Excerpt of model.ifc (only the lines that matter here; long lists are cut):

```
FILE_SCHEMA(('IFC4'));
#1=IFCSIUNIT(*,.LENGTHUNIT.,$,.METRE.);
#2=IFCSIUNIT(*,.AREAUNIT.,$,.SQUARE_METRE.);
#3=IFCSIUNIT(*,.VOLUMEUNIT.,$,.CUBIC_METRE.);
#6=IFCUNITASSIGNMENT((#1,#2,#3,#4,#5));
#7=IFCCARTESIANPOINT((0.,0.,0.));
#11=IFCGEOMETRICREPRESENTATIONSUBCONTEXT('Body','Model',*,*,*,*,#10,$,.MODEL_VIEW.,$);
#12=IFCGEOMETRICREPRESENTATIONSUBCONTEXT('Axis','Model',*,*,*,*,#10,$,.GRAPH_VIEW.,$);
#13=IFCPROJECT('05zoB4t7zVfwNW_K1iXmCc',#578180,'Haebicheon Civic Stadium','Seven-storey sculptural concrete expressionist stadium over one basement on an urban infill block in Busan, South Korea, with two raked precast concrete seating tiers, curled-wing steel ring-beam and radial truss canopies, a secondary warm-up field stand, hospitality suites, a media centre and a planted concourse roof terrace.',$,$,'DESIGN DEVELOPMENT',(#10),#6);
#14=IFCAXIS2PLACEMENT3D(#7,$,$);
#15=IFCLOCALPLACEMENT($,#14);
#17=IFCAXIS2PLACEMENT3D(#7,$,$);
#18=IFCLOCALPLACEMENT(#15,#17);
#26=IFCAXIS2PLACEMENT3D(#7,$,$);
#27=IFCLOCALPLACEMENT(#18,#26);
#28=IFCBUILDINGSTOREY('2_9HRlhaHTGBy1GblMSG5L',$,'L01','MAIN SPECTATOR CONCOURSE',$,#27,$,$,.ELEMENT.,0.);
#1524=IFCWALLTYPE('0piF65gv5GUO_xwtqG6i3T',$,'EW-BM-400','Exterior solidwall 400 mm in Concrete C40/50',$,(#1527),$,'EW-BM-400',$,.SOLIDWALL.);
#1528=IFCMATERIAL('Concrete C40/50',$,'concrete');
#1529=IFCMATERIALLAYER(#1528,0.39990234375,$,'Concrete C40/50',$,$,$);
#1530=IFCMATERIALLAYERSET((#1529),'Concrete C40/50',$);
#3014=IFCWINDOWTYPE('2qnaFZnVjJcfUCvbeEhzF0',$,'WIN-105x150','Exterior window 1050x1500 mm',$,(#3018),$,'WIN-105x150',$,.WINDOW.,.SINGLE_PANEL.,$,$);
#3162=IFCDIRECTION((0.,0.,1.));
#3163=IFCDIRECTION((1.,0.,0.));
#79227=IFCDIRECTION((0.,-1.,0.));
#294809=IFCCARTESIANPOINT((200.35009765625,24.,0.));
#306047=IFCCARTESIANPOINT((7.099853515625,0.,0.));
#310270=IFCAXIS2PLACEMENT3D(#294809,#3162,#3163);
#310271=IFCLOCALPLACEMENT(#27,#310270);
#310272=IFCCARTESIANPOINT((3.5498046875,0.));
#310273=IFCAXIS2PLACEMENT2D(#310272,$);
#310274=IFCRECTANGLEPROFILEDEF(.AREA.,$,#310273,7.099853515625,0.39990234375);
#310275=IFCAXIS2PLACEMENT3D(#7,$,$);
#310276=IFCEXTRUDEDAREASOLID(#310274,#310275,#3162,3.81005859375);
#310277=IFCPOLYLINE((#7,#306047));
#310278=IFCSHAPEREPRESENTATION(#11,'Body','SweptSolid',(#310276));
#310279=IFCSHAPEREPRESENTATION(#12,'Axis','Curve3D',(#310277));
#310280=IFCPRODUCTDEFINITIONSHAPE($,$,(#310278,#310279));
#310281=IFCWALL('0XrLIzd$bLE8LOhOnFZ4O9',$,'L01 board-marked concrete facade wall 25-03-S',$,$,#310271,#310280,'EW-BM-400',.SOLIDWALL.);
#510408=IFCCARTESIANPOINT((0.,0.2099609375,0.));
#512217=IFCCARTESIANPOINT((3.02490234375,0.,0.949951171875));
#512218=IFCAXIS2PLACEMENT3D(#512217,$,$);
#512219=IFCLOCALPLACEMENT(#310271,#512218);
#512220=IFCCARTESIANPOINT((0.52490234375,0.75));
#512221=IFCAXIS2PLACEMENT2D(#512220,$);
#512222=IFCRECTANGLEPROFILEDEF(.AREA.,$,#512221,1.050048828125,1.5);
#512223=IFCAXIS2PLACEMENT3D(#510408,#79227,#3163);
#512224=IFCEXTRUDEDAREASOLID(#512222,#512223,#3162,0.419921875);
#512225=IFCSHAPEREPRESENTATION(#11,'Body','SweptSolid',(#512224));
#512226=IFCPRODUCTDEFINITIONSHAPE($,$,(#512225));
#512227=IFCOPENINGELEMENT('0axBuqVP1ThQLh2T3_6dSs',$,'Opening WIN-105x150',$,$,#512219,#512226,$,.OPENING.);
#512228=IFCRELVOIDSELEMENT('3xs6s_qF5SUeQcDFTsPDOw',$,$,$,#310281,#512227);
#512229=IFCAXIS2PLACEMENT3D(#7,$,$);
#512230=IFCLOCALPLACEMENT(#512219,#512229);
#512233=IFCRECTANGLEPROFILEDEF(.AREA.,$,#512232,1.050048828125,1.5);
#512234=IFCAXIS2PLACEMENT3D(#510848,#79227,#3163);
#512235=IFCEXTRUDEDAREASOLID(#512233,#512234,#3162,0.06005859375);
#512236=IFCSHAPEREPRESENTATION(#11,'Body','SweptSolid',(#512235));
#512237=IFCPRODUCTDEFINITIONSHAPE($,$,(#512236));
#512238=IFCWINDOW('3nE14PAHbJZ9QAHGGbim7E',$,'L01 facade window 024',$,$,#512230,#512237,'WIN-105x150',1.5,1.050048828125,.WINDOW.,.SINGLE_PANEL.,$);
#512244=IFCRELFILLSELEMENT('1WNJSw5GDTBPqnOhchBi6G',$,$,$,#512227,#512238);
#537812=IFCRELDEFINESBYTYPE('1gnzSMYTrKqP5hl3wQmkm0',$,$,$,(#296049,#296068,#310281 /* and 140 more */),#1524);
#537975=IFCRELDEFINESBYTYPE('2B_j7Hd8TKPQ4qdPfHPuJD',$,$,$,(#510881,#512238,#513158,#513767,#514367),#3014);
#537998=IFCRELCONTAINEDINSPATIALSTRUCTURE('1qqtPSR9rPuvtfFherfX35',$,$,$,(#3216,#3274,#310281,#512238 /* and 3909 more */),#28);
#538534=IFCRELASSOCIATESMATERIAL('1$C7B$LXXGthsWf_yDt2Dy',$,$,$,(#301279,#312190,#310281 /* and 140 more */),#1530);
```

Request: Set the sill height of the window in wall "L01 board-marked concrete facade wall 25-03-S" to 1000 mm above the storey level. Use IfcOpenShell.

```python
import numpy as np
import ifcopenshell
import ifcopenshell.api.geometry
import ifcopenshell.geom
import ifcopenshell.util.element
import ifcopenshell.util.placement
import ifcopenshell.util.shape
import ifcopenshell.util.unit

model = ifcopenshell.open("model.ifc")
unit_scale = ifcopenshell.util.unit.calculate_unit_scale(model)

window = model.by_guid("3nE14PAHbJZ9QAHGGbim7E")
opening = window.FillsVoids[0].RelatingOpeningElement
storey = ifcopenshell.util.element.get_container(window, ifc_class="IfcBuildingStorey")
level = ifcopenshell.util.placement.get_local_placement(storey.ObjectPlacement)[2, 3]

# The opening's origin need not be at the sill, so measure its lowest point.
shape = ifcopenshell.geom.create_shape(ifcopenshell.geom.settings(), opening)
bottom = ifcopenshell.util.shape.get_shape_bottom_elevation(shape, shape.geometry) / unit_scale
dz = level + 1 / unit_scale - bottom

shift = np.array([0.0, 0.0, dz])
# The window is placed relative to its opening, so it follows when the opening moves.
matrix = ifcopenshell.util.placement.get_local_placement(opening.ObjectPlacement)
matrix[:3, 3] += shift
ifcopenshell.api.geometry.edit_object_placement(
    model, product=opening, matrix=matrix, is_si=False, should_transform_children=True
)

print(f"moved by {dz * unit_scale:+.3f} m")

model.write("model_rev.ifc")
```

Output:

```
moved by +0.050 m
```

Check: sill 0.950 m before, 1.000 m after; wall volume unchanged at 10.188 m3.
